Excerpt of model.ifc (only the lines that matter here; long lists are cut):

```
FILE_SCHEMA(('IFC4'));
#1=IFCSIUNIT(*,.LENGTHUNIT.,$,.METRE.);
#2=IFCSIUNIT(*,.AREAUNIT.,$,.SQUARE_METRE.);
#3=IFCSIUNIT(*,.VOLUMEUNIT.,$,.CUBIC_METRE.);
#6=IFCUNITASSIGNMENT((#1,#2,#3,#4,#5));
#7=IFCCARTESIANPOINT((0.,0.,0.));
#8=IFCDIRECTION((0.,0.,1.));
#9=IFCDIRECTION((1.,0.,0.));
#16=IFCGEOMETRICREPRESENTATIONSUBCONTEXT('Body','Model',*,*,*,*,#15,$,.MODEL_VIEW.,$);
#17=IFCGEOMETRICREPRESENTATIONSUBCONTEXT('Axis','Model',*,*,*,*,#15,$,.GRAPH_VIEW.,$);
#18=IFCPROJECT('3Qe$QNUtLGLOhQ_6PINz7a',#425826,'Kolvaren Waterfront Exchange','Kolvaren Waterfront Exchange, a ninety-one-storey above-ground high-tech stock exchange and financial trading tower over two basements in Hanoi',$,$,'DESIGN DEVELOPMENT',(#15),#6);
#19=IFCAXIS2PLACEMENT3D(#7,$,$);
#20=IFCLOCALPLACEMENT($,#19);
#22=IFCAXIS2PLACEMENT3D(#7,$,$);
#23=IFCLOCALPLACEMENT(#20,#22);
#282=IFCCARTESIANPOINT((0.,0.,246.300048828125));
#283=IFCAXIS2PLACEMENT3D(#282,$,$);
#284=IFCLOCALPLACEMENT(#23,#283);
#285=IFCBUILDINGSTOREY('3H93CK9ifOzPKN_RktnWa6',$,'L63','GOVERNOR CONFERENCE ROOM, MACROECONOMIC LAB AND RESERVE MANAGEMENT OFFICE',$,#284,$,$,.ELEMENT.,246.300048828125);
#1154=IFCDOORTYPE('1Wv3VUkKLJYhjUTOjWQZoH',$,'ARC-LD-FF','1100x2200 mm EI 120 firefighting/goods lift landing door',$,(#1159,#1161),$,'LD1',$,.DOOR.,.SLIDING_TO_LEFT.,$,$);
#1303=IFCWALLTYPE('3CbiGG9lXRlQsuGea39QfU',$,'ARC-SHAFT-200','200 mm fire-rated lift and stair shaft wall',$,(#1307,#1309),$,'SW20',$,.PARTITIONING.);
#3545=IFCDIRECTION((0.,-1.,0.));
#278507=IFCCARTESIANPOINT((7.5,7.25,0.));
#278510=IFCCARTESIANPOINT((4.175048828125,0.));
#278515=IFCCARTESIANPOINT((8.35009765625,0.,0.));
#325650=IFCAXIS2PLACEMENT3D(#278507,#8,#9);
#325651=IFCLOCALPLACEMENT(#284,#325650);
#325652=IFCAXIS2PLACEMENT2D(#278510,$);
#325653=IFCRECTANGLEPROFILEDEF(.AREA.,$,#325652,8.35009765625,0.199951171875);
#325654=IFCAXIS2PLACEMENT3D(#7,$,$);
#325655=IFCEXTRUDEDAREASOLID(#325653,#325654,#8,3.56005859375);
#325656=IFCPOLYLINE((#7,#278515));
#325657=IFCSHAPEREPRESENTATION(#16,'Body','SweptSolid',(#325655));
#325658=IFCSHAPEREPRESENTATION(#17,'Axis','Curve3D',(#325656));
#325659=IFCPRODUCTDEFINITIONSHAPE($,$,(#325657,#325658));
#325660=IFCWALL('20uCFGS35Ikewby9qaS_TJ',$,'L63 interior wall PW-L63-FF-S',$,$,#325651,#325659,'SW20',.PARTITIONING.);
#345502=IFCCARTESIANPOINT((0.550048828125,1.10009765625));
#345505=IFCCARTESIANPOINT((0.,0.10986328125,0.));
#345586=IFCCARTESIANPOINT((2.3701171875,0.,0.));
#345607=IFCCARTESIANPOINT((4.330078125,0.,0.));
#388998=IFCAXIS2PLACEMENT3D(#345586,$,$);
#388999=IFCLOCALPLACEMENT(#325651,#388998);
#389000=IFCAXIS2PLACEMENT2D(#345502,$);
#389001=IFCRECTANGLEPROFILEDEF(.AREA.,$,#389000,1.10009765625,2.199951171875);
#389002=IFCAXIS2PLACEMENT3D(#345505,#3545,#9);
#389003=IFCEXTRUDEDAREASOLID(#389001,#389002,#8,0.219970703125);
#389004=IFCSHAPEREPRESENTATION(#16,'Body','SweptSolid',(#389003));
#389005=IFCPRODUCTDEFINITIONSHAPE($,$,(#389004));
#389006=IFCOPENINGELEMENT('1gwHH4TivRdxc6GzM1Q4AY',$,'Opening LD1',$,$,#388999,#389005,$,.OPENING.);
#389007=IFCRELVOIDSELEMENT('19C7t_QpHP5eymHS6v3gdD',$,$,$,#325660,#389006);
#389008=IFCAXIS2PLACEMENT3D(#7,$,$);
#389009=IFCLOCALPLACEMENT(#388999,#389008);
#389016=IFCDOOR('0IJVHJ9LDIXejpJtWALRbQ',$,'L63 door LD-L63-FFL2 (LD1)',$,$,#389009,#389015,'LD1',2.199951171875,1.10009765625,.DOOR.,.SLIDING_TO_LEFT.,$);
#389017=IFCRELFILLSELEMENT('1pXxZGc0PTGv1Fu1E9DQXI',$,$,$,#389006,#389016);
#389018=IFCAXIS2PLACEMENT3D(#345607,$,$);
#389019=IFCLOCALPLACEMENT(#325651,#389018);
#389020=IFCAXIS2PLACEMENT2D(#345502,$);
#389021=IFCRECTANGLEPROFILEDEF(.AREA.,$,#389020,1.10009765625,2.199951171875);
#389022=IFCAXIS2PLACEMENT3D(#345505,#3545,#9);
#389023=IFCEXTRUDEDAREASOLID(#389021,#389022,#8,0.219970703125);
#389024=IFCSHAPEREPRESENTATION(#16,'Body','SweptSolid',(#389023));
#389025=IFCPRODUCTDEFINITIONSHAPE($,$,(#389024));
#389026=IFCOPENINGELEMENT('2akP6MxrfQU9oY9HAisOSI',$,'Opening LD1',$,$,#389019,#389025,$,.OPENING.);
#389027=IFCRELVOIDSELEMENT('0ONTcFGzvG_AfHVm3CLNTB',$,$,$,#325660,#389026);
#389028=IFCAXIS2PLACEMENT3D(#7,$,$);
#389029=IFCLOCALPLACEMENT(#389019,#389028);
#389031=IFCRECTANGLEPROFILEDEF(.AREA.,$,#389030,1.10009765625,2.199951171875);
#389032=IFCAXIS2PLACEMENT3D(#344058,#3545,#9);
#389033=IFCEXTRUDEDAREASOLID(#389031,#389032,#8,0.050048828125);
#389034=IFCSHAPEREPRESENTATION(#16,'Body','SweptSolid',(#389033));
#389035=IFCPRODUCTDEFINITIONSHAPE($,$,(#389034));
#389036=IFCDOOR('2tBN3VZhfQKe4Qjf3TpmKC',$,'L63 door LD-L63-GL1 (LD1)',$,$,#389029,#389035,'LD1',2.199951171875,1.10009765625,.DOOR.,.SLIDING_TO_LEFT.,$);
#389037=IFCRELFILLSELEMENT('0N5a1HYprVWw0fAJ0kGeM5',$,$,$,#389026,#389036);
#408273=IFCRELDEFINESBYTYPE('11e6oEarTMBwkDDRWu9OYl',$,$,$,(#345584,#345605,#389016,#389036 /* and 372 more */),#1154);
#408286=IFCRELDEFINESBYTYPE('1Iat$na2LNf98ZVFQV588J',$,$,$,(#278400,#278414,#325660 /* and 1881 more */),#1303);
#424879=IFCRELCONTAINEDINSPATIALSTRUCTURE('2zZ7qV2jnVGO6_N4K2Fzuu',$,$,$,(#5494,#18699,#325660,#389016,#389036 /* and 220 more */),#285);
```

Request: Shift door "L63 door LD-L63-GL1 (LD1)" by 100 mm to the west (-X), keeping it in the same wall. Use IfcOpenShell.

```python
import ifcopenshell
import ifcopenshell.api.geometry
import ifcopenshell.util.placement
import ifcopenshell.util.unit

model = ifcopenshell.open("model.ifc")
unit_scale = ifcopenshell.util.unit.calculate_unit_scale(model)

door = model.by_guid("2tBN3VZhfQKe4Qjf3TpmKC")
opening = door.FillsVoids[0].RelatingOpeningElement
wall = opening.VoidsElements[0].RelatingBuildingElement

wall_matrix = ifcopenshell.util.placement.get_local_placement(wall.ObjectPlacement)
shift = wall_matrix[:3, 0] * -0.1 / unit_scale
before = ifcopenshell.util.placement.get_local_placement(door.ObjectPlacement)[:3, 3].copy()

# The door is placed relative to its opening, so it follows when the opening moves.
matrix = ifcopenshell.util.placement.get_local_placement(opening.ObjectPlacement)
matrix[:3, 3] += shift
ifcopenshell.api.geometry.edit_object_placement(
    model, product=opening, matrix=matrix, is_si=False, should_transform_children=True
)

after = ifcopenshell.util.placement.get_local_placement(door.ObjectPlacement)[:3, 3]
print("door moved by", (after - before).round(3) + 0.0)

model.write("model_edited.ifc")
```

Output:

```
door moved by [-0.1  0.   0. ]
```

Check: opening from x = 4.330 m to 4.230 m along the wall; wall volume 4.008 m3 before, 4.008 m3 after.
